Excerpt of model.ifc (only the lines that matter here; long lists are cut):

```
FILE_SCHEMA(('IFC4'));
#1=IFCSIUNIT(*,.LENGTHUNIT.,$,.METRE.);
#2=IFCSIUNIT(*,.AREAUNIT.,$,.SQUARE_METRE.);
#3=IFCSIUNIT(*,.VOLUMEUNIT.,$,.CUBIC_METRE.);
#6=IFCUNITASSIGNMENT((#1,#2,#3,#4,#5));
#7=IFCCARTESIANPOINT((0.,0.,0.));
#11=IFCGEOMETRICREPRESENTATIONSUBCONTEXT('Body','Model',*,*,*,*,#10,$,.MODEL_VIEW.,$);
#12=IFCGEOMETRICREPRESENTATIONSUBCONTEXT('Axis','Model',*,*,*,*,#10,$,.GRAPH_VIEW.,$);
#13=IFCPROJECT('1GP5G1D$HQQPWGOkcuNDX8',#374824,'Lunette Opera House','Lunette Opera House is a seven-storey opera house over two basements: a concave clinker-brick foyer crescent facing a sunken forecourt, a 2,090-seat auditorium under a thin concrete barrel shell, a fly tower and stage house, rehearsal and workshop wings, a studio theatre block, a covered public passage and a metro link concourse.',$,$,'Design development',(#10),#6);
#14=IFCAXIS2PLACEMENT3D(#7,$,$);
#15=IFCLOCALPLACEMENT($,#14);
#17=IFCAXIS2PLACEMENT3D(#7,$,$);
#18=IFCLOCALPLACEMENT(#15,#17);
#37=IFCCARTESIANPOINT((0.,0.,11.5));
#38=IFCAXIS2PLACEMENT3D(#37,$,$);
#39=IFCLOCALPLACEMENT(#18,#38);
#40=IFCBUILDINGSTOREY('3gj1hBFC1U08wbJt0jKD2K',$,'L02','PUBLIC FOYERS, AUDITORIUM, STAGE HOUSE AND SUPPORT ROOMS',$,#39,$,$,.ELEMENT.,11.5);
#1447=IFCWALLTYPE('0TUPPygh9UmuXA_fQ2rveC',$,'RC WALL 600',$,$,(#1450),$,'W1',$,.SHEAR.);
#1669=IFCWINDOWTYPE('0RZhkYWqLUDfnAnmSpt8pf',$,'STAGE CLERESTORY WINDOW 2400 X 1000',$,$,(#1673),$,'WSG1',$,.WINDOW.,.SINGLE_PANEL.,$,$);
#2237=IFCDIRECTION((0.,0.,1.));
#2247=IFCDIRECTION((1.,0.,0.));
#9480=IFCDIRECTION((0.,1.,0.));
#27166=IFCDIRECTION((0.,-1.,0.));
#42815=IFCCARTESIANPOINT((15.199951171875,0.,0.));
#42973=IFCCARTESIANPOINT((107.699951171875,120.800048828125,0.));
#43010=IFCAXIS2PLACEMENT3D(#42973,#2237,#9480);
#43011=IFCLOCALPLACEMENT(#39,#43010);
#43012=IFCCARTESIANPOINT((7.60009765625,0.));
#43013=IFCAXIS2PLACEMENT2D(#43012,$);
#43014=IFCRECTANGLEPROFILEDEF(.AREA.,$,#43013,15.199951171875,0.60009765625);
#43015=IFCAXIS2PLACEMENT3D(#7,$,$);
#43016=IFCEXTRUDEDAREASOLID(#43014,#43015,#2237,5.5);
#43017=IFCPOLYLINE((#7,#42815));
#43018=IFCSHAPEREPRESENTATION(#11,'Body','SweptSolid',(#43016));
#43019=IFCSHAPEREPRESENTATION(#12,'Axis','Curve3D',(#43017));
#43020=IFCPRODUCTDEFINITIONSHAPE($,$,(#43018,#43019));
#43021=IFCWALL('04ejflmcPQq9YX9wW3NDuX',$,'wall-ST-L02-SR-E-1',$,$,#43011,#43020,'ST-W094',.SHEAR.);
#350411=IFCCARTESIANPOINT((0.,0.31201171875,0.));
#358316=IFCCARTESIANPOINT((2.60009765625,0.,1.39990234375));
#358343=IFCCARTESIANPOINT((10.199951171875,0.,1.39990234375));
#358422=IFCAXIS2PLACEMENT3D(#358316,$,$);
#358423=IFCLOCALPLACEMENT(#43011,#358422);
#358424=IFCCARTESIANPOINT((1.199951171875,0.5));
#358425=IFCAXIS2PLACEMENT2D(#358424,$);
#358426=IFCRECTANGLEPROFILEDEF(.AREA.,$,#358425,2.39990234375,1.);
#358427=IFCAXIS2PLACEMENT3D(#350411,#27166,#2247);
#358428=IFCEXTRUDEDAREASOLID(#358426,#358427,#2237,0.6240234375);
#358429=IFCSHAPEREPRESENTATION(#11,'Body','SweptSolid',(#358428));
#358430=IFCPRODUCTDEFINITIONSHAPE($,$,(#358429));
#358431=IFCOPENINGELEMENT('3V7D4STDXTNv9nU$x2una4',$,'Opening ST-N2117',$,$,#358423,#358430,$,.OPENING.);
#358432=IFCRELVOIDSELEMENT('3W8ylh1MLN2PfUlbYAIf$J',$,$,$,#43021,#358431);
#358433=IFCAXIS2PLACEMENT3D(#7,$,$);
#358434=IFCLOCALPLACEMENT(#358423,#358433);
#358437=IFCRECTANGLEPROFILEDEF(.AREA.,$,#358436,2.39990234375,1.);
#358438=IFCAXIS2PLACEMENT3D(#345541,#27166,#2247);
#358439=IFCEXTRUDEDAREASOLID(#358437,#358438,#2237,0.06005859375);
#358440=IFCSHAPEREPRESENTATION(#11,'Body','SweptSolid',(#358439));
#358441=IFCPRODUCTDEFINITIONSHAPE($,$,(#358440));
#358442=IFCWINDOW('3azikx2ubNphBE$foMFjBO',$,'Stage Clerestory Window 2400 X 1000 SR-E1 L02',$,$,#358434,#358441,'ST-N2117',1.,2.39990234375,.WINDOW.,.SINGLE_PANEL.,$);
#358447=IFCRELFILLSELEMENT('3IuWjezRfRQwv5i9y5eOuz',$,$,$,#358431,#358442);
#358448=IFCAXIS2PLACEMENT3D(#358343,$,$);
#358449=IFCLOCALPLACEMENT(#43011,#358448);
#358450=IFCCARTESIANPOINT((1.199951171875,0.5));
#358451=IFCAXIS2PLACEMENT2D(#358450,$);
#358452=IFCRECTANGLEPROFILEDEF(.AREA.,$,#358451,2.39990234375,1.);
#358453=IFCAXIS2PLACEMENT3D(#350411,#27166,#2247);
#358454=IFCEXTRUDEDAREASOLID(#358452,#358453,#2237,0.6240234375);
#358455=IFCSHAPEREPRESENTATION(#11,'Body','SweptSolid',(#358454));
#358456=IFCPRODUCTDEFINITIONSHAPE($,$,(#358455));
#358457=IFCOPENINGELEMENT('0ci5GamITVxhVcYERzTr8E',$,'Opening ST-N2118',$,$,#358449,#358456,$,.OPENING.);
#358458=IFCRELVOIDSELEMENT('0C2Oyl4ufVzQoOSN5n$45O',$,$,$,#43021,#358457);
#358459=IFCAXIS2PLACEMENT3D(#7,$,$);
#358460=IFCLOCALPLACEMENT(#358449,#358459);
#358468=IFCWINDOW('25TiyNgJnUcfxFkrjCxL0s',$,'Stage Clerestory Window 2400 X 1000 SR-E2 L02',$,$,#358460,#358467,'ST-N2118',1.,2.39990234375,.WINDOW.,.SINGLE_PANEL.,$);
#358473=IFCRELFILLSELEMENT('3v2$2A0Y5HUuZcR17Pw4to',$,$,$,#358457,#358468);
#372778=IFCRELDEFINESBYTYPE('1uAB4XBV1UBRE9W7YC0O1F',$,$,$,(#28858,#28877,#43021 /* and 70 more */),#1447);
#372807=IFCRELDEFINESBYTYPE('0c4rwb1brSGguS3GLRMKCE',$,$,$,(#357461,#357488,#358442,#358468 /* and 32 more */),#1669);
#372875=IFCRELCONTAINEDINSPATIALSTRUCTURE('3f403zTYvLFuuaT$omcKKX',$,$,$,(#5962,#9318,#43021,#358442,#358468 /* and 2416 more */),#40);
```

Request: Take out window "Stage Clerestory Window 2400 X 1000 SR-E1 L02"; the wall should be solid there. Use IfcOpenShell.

```python
import ifcopenshell
import ifcopenshell.api.feature
import ifcopenshell.api.root
import ifcopenshell.geom
import ifcopenshell.util.shape

model = ifcopenshell.open("model.ifc")
settings = ifcopenshell.geom.settings()


def volume(element):
    """Net volume in cubic metres, openings subtracted."""
    shape = ifcopenshell.geom.create_shape(settings, element)
    return ifcopenshell.util.shape.get_volume(shape.geometry)


window = model.by_guid("3azikx2ubNphBE$foMFjBO")
opening = window.FillsVoids[0].RelatingOpeningElement
wall = opening.VoidsElements[0].RelatingBuildingElement
before = volume(wall)

ifcopenshell.api.root.remove_product(model, product=window)
ifcopenshell.api.feature.remove_feature(model, feature=opening)

after = volume(wall)

print(f"wall volume {before:.3f} -> {after:.3f} m3")

model.write("model_rev.ifc")
```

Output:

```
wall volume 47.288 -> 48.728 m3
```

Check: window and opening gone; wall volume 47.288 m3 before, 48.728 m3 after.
